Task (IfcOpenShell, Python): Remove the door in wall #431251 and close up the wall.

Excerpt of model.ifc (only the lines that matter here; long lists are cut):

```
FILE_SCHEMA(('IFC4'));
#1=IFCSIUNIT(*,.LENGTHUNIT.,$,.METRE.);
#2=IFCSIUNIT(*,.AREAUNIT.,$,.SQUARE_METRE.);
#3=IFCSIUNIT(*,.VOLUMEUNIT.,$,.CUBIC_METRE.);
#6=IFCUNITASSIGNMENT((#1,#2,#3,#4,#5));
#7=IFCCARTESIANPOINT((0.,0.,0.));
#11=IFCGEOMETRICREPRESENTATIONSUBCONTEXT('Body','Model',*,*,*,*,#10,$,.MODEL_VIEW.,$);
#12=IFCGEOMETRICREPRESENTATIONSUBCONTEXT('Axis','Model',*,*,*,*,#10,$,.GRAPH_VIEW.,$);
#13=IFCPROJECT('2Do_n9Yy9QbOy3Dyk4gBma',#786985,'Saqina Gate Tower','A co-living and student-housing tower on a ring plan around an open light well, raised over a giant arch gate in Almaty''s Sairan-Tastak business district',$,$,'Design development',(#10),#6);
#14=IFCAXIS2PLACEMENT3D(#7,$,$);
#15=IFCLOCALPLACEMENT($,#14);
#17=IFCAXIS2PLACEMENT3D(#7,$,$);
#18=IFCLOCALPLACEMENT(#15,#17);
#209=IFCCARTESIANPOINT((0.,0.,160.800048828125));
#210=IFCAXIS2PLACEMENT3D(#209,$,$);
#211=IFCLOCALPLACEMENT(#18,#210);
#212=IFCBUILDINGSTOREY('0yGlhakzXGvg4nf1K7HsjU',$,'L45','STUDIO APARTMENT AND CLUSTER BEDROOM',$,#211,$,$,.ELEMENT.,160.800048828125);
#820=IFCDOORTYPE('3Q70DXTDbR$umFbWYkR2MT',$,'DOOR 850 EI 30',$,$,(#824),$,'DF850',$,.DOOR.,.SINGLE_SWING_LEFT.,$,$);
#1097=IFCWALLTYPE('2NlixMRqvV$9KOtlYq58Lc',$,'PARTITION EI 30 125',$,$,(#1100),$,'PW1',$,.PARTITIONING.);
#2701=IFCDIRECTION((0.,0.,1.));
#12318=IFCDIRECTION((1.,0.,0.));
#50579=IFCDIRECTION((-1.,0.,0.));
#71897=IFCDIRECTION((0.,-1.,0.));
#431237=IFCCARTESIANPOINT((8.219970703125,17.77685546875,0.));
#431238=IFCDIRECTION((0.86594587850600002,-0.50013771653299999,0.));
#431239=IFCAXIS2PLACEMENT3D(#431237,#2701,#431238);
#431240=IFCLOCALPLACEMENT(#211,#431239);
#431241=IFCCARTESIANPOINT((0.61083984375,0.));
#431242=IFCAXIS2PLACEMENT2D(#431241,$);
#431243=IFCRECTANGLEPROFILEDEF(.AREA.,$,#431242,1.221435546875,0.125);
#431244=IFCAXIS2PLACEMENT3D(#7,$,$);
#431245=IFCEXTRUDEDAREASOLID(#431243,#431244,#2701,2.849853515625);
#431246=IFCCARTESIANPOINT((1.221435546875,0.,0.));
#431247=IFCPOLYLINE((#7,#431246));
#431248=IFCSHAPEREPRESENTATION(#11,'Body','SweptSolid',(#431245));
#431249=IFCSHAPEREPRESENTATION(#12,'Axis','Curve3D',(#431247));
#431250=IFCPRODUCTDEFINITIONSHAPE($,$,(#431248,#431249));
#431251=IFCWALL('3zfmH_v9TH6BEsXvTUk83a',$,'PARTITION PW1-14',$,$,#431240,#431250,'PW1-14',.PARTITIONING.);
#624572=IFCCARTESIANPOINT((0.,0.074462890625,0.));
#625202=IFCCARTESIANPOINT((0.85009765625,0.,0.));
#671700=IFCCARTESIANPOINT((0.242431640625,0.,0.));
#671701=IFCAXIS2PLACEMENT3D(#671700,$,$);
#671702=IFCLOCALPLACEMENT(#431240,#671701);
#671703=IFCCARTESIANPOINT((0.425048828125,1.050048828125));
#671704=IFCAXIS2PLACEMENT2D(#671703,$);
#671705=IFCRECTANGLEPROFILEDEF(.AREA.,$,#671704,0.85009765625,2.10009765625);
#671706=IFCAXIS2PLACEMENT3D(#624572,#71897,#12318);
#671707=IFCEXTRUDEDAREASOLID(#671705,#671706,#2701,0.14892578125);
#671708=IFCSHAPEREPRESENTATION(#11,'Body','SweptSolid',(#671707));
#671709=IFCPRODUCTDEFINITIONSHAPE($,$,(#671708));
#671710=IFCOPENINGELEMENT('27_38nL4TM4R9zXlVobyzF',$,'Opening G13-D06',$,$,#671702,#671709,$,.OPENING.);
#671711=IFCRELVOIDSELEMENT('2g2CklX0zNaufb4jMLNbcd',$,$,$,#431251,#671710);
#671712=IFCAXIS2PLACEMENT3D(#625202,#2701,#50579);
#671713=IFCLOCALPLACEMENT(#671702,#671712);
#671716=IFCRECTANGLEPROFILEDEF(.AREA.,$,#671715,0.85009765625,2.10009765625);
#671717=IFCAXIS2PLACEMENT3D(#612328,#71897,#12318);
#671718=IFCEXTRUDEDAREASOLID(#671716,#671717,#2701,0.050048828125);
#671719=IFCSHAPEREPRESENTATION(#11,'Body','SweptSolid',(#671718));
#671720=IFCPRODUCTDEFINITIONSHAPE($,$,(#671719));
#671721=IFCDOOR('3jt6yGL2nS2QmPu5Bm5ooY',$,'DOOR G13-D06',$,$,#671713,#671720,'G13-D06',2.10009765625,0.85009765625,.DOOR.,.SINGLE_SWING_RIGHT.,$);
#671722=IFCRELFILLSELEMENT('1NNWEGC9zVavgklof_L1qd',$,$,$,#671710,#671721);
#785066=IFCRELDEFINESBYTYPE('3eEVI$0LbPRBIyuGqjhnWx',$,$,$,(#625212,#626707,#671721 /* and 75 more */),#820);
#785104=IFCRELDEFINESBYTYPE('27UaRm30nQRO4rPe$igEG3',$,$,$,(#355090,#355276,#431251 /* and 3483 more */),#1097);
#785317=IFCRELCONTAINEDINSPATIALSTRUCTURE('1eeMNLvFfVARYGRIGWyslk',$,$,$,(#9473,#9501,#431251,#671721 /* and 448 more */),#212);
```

```python
import ifcopenshell
import ifcopenshell.api.feature
import ifcopenshell.api.root
import ifcopenshell.geom
import ifcopenshell.util.shape

model = ifcopenshell.open("model.ifc")
settings = ifcopenshell.geom.settings()


def volume(element):
    """Net volume in cubic metres, openings subtracted."""
    shape = ifcopenshell.geom.create_shape(settings, element)
    return ifcopenshell.util.shape.get_volume(shape.geometry)


door = model.by_guid("3jt6yGL2nS2QmPu5Bm5ooY")
opening = door.FillsVoids[0].RelatingOpeningElement
wall = opening.VoidsElements[0].RelatingBuildingElement
before = volume(wall)

ifcopenshell.api.root.remove_product(model, product=door)
ifcopenshell.api.feature.remove_feature(model, feature=opening)

after = volume(wall)

print(f"wall volume {before:.3f} -> {after:.3f} m3")

model.write("model_rev.ifc")
```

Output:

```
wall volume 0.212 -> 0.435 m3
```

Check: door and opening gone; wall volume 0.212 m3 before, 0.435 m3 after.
